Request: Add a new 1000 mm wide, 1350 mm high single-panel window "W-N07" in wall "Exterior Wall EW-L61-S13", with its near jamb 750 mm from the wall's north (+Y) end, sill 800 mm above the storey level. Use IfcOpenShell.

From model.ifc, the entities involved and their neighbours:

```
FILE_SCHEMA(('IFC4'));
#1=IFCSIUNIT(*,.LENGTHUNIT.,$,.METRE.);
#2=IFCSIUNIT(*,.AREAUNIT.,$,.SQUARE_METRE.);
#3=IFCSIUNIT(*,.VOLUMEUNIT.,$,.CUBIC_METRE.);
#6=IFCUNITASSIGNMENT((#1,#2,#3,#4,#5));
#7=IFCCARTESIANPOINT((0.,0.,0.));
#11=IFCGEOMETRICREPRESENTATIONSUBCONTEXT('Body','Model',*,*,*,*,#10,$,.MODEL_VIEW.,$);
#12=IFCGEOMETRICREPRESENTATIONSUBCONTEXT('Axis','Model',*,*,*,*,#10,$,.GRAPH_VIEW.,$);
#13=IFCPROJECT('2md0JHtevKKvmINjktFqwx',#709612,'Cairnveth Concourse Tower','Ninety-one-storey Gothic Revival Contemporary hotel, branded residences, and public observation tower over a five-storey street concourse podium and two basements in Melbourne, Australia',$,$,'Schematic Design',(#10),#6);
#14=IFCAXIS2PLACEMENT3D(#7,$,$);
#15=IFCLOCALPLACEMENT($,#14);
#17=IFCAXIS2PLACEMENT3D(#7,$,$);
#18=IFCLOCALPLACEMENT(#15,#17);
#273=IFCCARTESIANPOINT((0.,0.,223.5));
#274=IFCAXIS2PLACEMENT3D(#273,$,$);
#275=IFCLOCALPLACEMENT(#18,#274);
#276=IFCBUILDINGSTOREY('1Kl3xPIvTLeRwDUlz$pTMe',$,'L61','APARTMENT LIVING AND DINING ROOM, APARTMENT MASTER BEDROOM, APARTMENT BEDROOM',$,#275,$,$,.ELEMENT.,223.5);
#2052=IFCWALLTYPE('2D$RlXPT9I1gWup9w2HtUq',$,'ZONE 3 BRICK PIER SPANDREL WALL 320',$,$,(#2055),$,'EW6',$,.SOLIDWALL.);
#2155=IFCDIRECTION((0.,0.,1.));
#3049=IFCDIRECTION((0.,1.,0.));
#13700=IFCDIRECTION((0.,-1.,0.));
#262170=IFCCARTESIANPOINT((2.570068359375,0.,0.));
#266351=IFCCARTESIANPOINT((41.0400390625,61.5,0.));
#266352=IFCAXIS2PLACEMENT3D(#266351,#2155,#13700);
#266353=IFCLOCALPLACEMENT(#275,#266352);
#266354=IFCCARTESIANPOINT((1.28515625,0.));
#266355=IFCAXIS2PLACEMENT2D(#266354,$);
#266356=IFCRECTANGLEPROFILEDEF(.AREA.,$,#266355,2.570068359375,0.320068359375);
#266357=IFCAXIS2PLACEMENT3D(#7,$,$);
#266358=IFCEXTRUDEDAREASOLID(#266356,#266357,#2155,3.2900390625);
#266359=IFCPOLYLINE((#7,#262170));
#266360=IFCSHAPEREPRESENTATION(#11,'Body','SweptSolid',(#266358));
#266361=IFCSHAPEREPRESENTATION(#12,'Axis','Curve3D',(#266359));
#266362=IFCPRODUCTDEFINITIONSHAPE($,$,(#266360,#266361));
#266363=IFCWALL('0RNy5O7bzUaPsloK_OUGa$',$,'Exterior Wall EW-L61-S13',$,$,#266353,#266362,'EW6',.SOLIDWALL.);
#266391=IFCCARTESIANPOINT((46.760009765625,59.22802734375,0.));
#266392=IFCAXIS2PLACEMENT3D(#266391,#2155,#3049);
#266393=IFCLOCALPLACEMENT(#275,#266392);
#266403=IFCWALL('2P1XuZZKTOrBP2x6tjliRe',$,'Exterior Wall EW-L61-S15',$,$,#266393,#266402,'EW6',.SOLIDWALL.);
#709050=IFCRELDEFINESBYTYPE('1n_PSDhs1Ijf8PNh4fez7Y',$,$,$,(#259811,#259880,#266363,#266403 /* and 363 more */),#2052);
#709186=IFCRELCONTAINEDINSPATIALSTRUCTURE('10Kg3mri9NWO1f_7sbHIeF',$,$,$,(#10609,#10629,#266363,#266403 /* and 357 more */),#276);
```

```python
import numpy as np
import ifcopenshell
import ifcopenshell.api.feature
import ifcopenshell.api.geometry
import ifcopenshell.api.root
import ifcopenshell.api.spatial
import ifcopenshell.geom
import ifcopenshell.util.element
import ifcopenshell.util.placement
import ifcopenshell.util.representation
import ifcopenshell.util.shape
import ifcopenshell.util.unit

model = ifcopenshell.open("model.ifc")
unit_scale = ifcopenshell.util.unit.calculate_unit_scale(model)
settings = ifcopenshell.geom.settings()


def volume(element):
    """Net volume in cubic metres, openings subtracted."""
    shape = ifcopenshell.geom.create_shape(settings, element)
    return ifcopenshell.util.shape.get_volume(shape.geometry)


wall = model.by_guid("0RNy5O7bzUaPsloK_OUGa$")
storey = ifcopenshell.util.element.get_container(wall, ifc_class="IfcBuildingStorey")
context = ifcopenshell.util.representation.get_context(model, "Model", "Body", "MODEL_VIEW")
before = volume(wall)

width, height, from_end, sill = 1, 1.35, 0.75, 0.8  # metres

# The wall runs along its own X axis, and the end named is its -X end.
wall_shape = ifcopenshell.geom.create_shape(settings, wall)
x, y, z = ifcopenshell.util.shape.get_vertices(wall_shape.geometry).T
start = x.min() + from_end
face, thickness = float(y.min()), float(y.max() - y.min())
wall_matrix = ifcopenshell.util.placement.get_local_placement(wall.ObjectPlacement)
level = ifcopenshell.util.placement.get_local_placement(storey.ObjectPlacement)[2, 3]


def in_wall(x, y):
    """Placement at x, y metres in the wall's axes, at sill height."""
    matrix = wall_matrix.copy()
    matrix[:, 3] = wall_matrix @ np.array([x / unit_scale, y / unit_scale, 0.0, 1.0])
    matrix[2, 3] = level + sill / unit_scale
    return matrix


# Opening: a box that overshoots both wall faces by 50 mm.
opening = ifcopenshell.api.root.create_entity(model, ifc_class="IfcOpeningElement", predefined_type="OPENING")
box = ifcopenshell.api.geometry.add_wall_representation(
    model, context=context, length=width, height=height, thickness=thickness + 0.1
)
ifcopenshell.api.geometry.assign_representation(model, product=opening, representation=box)
ifcopenshell.api.geometry.edit_object_placement(model, product=opening, matrix=in_wall(start, face - 0.05), is_si=False)
ifcopenshell.api.feature.add_feature(model, feature=opening, element=wall)

window = ifcopenshell.api.root.create_entity(model, ifc_class="IfcWindow", name="W-N07", predefined_type="WINDOW")
window.OverallWidth, window.OverallHeight = width / unit_scale, height / unit_scale
window.PartitioningType = "SINGLE_PANEL"
body = ifcopenshell.api.geometry.add_window_representation(
    model,
    context=context,
    overall_width=window.OverallWidth,
    overall_height=window.OverallHeight,
    partition_type="SINGLE_PANEL",
)
ifcopenshell.api.geometry.assign_representation(model, product=window, representation=body)
ifcopenshell.api.spatial.assign_container(model, products=[window], relating_structure=storey)
ifcopenshell.api.feature.add_filling(model, opening=opening, element=window)

# Centre the window in the wall's thickness.
ifcopenshell.api.geometry.edit_object_placement(model, product=window, matrix=in_wall(start, face), is_si=False)
window_shape = ifcopenshell.geom.create_shape(settings, window)
depth = ifcopenshell.util.shape.get_vertices(window_shape.geometry)[:, 1]
offset = face + thickness / 2 - (depth.min() + depth.max()) / 2
ifcopenshell.api.geometry.edit_object_placement(model, product=window, matrix=in_wall(start, offset), is_si=False)

after = volume(wall)

print(f"wall volume {before:.3f} -> {after:.3f} m3")

model.write("model_rev.ifc")
```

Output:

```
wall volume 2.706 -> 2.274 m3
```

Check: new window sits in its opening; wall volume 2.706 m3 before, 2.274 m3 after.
